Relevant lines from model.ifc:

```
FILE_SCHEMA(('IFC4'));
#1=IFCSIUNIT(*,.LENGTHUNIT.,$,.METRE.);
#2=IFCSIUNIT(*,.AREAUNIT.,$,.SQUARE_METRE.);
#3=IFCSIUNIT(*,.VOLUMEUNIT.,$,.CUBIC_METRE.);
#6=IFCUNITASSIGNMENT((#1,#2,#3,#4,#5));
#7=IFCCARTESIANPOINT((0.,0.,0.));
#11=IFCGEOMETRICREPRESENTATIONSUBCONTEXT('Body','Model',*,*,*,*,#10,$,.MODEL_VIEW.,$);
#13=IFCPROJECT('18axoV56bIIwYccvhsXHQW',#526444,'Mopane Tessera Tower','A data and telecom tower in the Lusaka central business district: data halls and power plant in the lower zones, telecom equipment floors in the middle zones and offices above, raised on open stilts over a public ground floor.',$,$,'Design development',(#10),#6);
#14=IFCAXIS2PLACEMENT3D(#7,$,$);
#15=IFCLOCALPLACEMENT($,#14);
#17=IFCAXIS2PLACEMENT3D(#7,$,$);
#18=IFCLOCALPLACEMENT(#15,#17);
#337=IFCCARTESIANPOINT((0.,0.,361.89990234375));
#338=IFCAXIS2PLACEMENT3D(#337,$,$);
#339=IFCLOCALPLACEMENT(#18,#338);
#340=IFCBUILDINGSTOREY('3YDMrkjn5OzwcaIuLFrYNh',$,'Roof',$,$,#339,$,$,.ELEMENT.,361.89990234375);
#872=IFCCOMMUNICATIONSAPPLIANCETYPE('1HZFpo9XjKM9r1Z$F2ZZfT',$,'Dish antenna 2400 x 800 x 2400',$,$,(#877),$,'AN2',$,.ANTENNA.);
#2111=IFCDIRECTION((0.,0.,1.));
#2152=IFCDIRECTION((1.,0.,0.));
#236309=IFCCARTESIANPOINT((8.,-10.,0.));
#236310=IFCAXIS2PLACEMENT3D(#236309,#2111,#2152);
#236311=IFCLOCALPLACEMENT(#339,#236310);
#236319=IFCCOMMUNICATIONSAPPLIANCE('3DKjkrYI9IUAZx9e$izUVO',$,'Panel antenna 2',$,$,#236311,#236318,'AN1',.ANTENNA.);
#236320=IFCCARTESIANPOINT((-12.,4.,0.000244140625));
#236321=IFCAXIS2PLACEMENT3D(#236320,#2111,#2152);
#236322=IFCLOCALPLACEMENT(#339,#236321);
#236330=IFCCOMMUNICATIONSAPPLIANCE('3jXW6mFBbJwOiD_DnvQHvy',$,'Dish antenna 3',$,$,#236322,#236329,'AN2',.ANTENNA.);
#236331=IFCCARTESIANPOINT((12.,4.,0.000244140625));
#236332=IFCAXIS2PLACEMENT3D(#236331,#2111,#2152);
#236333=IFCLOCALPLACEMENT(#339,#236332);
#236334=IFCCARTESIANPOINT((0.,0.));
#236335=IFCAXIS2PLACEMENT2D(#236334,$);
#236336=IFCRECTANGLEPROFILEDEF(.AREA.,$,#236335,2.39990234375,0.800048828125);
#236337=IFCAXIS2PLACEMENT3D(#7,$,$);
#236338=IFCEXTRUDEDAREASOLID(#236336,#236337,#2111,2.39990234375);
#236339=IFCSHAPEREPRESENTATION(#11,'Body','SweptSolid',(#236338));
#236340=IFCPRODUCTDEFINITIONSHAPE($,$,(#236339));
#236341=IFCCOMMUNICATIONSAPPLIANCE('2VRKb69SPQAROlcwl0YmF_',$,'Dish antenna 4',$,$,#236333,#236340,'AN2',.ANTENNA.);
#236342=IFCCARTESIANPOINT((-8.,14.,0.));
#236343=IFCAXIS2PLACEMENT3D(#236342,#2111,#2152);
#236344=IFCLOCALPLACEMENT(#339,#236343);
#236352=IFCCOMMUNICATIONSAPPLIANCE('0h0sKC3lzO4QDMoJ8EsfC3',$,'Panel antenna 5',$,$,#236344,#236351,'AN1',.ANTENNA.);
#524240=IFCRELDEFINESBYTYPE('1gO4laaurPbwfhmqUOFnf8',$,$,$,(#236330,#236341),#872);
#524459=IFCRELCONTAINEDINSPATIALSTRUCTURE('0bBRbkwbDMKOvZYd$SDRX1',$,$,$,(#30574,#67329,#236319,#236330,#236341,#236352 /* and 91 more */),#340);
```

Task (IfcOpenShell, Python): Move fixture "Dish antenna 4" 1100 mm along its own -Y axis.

```python
import ifcopenshell
import ifcopenshell.api.geometry
import ifcopenshell.util.placement
import ifcopenshell.util.unit

model = ifcopenshell.open("model.ifc")
unit_scale = ifcopenshell.util.unit.calculate_unit_scale(model)

item = model.by_guid("2VRKb69SPQAROlcwl0YmF_")
matrix = ifcopenshell.util.placement.get_local_placement(item.ObjectPlacement)
matrix[:3, 3] -= matrix[:3, 1] * 1.1 / unit_scale
ifcopenshell.api.geometry.edit_object_placement(model, product=item, matrix=matrix, is_si=False)

print(ifcopenshell.util.placement.get_local_placement(item.ObjectPlacement).round(3) + 0.0)

model.write("model-out.ifc")
```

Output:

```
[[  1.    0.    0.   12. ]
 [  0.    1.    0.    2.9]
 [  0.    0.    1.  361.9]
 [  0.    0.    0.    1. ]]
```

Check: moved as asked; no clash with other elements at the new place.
